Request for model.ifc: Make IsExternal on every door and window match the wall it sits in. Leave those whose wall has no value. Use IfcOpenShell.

First a look at what the model holds.

```python
import ifcopenshell
import ifcopenshell.util.element

model = ifcopenshell.open("model.ifc")
print(model.schema)
seen = {}
for e in model.by_type("IfcDoor") + model.by_type("IfcWindow"):
    if not e.FillsVoids:
        continue
    host = e.FillsVoids[0].RelatingOpeningElement.VoidsElements[0].RelatingBuildingElement
    own = ifcopenshell.util.element.get_pset(e, f"Pset_{e.is_a()[3:].removesuffix('StandardCase')}Common", "IsExternal")
    wall = ifcopenshell.util.element.get_pset(host, "Pset_WallCommon", "IsExternal")
    seen[e.is_a(), own, wall] = seen.get((e.is_a(), own, wall), 0) + 1
for (cls, own, wall), count in sorted(seen.items(), key=str):
    print(count, cls, "IsExternal:", own, "| host wall:", wall)
```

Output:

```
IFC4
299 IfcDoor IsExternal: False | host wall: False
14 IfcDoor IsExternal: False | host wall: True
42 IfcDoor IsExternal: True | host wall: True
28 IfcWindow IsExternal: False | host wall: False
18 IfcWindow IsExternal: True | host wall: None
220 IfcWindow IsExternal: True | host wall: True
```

```python
import ifcopenshell
import ifcopenshell.api.pset
import ifcopenshell.util.element

model = ifcopenshell.open("model.ifc")

count = 0
for ifc_class, pset_name in (("IfcDoor", "Pset_DoorCommon"), ("IfcWindow", "Pset_WindowCommon")):
    for e in model.by_type(ifc_class):
        if not e.FillsVoids:
            continue
        host = e.FillsVoids[0].RelatingOpeningElement.VoidsElements[0].RelatingBuildingElement
        external = ifcopenshell.util.element.get_pset(host, "Pset_WallCommon", "IsExternal")
        if external is None or ifcopenshell.util.element.get_pset(e, pset_name, "IsExternal") == external:
            continue
        pset = ifcopenshell.api.pset.add_pset(model, product=e, name=pset_name)
        ifcopenshell.api.pset.edit_pset(model, pset=pset, properties={"IsExternal": external})
        count += 1

print(count, "updated")

model.write("model_edited.ifc")
```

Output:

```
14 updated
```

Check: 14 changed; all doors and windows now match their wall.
